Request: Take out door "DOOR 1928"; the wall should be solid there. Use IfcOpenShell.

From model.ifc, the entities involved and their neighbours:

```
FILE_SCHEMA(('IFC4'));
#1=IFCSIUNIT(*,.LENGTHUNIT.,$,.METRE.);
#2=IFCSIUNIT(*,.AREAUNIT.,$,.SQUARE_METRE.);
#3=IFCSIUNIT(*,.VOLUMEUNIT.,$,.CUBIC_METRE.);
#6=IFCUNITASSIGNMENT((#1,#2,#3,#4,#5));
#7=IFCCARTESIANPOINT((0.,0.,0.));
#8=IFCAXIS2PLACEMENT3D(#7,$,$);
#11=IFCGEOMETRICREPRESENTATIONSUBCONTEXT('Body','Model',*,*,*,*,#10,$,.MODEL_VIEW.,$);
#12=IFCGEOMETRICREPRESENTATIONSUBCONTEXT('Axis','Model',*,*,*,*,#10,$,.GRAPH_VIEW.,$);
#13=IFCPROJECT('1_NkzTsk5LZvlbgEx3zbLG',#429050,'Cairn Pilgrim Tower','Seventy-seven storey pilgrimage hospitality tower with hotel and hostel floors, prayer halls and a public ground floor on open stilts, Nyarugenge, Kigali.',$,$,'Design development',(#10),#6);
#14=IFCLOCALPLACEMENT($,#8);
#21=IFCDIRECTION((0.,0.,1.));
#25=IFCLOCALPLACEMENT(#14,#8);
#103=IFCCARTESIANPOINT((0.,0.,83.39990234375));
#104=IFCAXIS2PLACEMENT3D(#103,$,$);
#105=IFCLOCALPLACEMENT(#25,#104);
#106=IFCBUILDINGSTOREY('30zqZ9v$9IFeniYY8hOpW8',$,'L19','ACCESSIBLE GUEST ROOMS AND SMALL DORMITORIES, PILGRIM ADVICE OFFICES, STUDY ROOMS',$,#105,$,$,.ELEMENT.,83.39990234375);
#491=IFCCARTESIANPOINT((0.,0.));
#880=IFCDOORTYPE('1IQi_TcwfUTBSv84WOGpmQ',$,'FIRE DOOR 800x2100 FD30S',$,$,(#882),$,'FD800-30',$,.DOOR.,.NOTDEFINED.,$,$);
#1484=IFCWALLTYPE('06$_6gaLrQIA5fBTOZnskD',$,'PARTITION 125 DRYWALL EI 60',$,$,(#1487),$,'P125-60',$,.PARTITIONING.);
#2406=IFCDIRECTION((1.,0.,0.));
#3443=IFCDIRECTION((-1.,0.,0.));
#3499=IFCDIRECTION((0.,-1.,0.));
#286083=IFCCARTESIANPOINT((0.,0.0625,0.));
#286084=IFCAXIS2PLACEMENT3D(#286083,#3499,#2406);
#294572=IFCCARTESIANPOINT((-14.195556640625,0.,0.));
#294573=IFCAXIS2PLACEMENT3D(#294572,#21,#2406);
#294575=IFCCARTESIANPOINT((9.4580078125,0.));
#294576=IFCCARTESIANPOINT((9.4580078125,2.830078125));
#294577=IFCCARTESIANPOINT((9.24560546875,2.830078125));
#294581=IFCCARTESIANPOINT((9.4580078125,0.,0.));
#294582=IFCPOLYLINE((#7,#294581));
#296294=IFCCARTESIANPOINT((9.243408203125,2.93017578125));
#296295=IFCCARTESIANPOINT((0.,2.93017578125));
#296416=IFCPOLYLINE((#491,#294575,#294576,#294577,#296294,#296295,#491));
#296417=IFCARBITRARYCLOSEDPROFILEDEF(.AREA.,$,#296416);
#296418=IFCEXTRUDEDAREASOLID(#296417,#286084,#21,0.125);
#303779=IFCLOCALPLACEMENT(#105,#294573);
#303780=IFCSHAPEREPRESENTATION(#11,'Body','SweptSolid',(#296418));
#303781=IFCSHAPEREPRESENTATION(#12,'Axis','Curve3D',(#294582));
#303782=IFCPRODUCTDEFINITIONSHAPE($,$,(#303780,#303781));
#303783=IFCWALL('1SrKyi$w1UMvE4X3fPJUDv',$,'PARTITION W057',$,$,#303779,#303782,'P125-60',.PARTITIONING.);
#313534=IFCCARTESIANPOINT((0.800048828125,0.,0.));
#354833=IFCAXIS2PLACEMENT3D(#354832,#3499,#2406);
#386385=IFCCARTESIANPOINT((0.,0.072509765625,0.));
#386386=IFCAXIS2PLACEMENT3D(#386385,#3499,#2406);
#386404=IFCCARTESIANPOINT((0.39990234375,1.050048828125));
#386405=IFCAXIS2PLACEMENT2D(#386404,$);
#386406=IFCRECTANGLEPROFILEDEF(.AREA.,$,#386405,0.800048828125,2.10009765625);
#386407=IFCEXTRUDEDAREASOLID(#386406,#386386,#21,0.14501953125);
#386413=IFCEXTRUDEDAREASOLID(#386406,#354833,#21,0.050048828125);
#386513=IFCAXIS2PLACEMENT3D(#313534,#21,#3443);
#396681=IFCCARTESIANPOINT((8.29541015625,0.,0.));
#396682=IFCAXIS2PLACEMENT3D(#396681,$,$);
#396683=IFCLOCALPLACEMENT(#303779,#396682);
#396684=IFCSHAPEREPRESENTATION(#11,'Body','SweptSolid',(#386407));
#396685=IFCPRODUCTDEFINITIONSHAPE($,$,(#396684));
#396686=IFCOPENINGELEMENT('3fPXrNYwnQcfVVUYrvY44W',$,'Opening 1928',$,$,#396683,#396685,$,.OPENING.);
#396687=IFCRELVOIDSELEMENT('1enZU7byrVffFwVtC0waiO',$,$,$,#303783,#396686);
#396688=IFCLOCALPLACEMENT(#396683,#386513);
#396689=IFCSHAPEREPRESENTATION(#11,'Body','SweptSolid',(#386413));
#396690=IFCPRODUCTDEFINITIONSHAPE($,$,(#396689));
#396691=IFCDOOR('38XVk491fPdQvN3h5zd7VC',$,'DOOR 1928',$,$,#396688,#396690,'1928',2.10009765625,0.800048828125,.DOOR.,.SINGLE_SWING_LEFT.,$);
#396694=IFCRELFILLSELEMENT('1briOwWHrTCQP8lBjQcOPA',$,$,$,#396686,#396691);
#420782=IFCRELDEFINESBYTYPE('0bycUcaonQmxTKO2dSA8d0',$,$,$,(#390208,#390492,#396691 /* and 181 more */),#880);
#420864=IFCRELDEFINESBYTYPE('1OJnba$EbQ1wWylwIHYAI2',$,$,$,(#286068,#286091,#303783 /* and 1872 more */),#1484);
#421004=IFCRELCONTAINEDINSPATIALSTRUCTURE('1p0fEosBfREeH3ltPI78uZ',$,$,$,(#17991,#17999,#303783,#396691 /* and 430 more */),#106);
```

```python
import ifcopenshell
import ifcopenshell.api.feature
import ifcopenshell.api.root
import ifcopenshell.geom
import ifcopenshell.util.shape

model = ifcopenshell.open("model.ifc")
settings = ifcopenshell.geom.settings()


def volume(element):
    """Net volume in cubic metres, openings subtracted."""
    shape = ifcopenshell.geom.create_shape(settings, element)
    return ifcopenshell.util.shape.get_volume(shape.geometry)


door = model.by_guid("38XVk491fPdQvN3h5zd7VC")
opening = door.FillsVoids[0].RelatingOpeningElement
wall = opening.VoidsElements[0].RelatingBuildingElement
before = volume(wall)

ifcopenshell.api.root.remove_product(model, product=door)
ifcopenshell.api.feature.remove_feature(model, feature=opening)

after = volume(wall)

print(f"wall volume {before:.3f} -> {after:.3f} m3")

model.write("model_rev.ifc")
```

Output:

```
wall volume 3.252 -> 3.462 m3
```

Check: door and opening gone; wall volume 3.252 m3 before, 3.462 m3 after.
